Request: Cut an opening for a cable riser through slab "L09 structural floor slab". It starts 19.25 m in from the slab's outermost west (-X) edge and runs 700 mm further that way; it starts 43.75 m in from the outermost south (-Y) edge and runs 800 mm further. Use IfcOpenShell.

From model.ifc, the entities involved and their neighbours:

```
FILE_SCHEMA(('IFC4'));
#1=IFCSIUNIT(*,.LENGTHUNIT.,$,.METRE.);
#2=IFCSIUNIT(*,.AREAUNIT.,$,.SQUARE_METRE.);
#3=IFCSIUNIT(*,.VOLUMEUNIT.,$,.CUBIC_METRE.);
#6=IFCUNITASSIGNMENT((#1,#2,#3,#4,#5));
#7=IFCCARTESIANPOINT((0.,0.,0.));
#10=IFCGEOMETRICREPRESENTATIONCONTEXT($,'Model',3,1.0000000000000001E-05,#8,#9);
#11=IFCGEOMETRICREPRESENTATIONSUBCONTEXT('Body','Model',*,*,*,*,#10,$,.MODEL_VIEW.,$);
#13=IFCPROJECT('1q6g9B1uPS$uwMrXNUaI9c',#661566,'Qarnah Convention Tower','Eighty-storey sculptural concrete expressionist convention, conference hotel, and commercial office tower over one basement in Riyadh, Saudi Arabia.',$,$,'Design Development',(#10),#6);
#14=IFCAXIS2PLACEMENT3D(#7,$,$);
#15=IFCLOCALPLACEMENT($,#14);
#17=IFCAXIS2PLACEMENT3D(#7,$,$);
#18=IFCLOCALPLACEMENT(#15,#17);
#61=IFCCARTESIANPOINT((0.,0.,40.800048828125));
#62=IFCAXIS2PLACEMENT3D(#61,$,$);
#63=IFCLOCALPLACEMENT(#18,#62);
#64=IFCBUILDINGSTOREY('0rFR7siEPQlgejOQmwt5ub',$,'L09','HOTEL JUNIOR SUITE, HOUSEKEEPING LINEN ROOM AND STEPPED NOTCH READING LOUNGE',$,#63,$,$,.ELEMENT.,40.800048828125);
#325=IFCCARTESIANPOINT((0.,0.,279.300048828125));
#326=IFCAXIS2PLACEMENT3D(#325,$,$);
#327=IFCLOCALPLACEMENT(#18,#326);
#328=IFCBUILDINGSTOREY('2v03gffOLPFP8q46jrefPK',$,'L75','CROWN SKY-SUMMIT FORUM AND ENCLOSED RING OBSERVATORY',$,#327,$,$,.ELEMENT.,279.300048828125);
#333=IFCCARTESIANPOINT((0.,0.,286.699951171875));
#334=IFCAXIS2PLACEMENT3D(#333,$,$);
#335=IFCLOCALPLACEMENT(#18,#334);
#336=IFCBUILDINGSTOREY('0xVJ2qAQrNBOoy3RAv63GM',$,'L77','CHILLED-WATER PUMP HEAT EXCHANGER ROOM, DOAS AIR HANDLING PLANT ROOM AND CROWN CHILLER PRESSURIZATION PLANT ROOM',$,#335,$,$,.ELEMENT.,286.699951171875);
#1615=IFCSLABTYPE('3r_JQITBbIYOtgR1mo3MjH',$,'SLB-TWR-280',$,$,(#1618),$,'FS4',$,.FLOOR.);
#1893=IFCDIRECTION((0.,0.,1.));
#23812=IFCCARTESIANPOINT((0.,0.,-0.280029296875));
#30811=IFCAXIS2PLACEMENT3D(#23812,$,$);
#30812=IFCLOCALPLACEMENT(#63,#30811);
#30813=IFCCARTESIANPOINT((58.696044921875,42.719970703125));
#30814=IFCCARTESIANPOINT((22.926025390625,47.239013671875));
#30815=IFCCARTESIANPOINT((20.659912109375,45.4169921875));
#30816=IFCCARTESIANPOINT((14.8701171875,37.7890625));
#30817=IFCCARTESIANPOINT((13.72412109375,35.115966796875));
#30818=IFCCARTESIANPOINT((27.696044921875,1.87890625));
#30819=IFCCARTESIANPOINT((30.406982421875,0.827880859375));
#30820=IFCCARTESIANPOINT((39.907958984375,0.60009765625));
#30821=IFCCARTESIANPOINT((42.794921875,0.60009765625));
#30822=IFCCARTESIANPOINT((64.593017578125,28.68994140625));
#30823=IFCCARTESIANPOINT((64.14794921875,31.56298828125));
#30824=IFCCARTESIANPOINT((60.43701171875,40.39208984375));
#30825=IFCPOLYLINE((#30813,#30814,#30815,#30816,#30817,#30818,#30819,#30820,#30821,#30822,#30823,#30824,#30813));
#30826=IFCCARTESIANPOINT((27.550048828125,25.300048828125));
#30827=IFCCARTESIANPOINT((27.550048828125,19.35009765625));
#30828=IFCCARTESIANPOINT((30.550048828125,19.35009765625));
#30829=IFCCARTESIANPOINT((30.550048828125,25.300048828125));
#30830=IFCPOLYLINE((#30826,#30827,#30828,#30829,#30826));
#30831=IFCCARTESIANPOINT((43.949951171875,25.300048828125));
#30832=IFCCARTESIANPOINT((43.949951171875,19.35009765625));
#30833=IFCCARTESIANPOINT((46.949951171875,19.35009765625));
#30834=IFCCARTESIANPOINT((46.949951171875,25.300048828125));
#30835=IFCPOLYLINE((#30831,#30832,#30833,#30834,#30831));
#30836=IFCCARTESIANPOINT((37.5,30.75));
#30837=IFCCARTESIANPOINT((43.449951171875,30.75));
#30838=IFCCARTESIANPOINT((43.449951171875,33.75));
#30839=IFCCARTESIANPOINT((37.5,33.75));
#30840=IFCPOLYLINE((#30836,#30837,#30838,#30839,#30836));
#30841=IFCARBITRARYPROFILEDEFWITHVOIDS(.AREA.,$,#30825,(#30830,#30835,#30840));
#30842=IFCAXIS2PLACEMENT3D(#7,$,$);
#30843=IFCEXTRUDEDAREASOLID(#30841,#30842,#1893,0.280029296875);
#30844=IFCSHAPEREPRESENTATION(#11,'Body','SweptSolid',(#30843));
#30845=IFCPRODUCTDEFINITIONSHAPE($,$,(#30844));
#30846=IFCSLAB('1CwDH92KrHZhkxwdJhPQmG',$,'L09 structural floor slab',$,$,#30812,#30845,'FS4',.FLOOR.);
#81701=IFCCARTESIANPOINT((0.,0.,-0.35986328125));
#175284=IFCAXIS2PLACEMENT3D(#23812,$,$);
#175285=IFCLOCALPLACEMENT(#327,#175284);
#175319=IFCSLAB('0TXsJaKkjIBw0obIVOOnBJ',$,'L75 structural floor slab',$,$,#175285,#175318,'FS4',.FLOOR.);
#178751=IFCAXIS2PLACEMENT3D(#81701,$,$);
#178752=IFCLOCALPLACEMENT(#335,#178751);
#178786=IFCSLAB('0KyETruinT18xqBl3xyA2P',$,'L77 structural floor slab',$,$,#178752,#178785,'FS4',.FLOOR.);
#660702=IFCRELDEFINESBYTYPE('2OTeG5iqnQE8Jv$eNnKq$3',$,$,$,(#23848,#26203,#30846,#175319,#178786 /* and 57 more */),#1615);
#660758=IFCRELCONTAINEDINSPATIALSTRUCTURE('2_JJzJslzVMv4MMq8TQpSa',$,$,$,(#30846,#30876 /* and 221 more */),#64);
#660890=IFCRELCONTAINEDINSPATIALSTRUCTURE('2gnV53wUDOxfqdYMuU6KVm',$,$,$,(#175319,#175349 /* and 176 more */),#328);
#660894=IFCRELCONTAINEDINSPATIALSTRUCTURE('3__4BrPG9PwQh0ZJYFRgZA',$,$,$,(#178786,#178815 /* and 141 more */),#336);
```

```python
import numpy as np
import ifcopenshell
import ifcopenshell.api.feature
import ifcopenshell.api.geometry
import ifcopenshell.api.root
import ifcopenshell.geom
import ifcopenshell.util.placement
import ifcopenshell.util.representation
import ifcopenshell.util.shape
import ifcopenshell.util.unit

model = ifcopenshell.open("model.ifc")
unit_scale = ifcopenshell.util.unit.calculate_unit_scale(model)
settings = ifcopenshell.geom.settings()


def volume(element):
    """Net volume in cubic metres, openings subtracted."""
    shape = ifcopenshell.geom.create_shape(settings, element)
    return ifcopenshell.util.shape.get_volume(shape.geometry)


slab = model.by_id(30846)
before = volume(slab)

# Extent in the slab's own axes, in metres. The edges named are its -X and -Y sides.
slab_shape = ifcopenshell.geom.create_shape(settings, slab)
vertices = ifcopenshell.util.shape.get_vertices(slab_shape.geometry)
x_min, y_min, bottom = vertices.min(axis=0)
top = vertices[:, 2].max()

opening = ifcopenshell.api.root.create_entity(model, ifc_class="IfcOpeningElement", name="Cable riser opening", predefined_type="OPENING")
context = ifcopenshell.util.representation.get_context(model, "Model", "Body", "MODEL_VIEW")
width, depth = 0.7, 0.8
outline = [(0.0, 0.0), (width, 0.0), (width, depth), (0.0, depth), (0.0, 0.0)]
# Overshoot both faces by 50 mm so the cut is clean.
shape = ifcopenshell.api.geometry.add_slab_representation(
    model, context=context, depth=top - bottom + 0.1, polyline=outline
)
ifcopenshell.api.geometry.assign_representation(model, product=opening, representation=shape)

matrix = ifcopenshell.util.placement.get_local_placement(slab.ObjectPlacement)
matrix[:, 3] = matrix @ np.append(np.array([x_min + 19.25, y_min + 43.75, bottom - 0.05]) / unit_scale, 1.0)
ifcopenshell.api.geometry.edit_object_placement(model, product=opening, matrix=matrix, is_si=False)
ifcopenshell.api.feature.add_feature(model, feature=opening, element=slab)

after = volume(slab)

print(f"slab volume {before:.3f} -> {after:.3f} m3")

model.write("model_rev.ifc")
```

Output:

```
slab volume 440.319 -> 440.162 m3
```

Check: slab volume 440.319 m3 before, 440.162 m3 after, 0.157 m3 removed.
